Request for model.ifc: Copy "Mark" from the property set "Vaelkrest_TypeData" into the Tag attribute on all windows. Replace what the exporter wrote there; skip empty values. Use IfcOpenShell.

First a look at what the model holds.

```python
import ifcopenshell
import ifcopenshell.util.element

model = ifcopenshell.open("model.ifc")
print(model.schema)
windows = model.by_type("IfcWindow")
print(len(windows), "windows")
for e in windows[:8]:
    source = ifcopenshell.util.element.get_pset(e, "Vaelkrest_TypeData", "Mark")
    target = e.Tag
    print(e.id(), repr(source), repr(target), sep=" | ")
```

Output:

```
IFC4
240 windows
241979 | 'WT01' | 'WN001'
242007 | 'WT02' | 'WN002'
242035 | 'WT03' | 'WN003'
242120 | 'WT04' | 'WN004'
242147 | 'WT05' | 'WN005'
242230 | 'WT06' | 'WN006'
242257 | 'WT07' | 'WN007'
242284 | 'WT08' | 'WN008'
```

```python
import ifcopenshell
import ifcopenshell.util.element

model = ifcopenshell.open("model.ifc")

count = 0
for e in model.by_type("IfcWindow"):
    value = ifcopenshell.util.element.get_pset(e, "Vaelkrest_TypeData", "Mark")
    current = e.Tag
    if not value or not value.strip() or current == value:
        continue
    e.Tag = value
    count += 1

print(count, "windows updated")

model.write("model_edited.ifc")
```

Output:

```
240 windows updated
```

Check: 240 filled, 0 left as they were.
